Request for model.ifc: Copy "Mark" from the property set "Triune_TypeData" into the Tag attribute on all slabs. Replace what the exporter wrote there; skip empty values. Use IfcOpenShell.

First a look at what the model holds.

```python
import ifcopenshell
import ifcopenshell.util.element

model = ifcopenshell.open("model.ifc")
print(model.schema)
slabs = model.by_type("IfcSlab")
print(len(slabs), "slabs")
for e in slabs[:8]:
    source = ifcopenshell.util.element.get_pset(e, "Triune_TypeData", "Mark")
    target = e.Tag
    print(e.id(), repr(source), repr(target), sep=" | ")
```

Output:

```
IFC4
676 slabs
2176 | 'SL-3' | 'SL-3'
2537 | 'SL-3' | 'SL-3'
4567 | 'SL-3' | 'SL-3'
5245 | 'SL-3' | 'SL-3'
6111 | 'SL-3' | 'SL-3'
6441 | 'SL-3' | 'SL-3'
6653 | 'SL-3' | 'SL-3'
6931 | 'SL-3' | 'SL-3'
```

```python
import ifcopenshell
import ifcopenshell.util.element

model = ifcopenshell.open("model.ifc")

count = 0
for e in model.by_type("IfcSlab"):
    value = ifcopenshell.util.element.get_pset(e, "Triune_TypeData", "Mark")
    current = e.Tag
    if not value or not value.strip() or current == value:
        continue
    e.Tag = value
    count += 1

print(count, "slabs updated")

model.write("model-out.ifc")
```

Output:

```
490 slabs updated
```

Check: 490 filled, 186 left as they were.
